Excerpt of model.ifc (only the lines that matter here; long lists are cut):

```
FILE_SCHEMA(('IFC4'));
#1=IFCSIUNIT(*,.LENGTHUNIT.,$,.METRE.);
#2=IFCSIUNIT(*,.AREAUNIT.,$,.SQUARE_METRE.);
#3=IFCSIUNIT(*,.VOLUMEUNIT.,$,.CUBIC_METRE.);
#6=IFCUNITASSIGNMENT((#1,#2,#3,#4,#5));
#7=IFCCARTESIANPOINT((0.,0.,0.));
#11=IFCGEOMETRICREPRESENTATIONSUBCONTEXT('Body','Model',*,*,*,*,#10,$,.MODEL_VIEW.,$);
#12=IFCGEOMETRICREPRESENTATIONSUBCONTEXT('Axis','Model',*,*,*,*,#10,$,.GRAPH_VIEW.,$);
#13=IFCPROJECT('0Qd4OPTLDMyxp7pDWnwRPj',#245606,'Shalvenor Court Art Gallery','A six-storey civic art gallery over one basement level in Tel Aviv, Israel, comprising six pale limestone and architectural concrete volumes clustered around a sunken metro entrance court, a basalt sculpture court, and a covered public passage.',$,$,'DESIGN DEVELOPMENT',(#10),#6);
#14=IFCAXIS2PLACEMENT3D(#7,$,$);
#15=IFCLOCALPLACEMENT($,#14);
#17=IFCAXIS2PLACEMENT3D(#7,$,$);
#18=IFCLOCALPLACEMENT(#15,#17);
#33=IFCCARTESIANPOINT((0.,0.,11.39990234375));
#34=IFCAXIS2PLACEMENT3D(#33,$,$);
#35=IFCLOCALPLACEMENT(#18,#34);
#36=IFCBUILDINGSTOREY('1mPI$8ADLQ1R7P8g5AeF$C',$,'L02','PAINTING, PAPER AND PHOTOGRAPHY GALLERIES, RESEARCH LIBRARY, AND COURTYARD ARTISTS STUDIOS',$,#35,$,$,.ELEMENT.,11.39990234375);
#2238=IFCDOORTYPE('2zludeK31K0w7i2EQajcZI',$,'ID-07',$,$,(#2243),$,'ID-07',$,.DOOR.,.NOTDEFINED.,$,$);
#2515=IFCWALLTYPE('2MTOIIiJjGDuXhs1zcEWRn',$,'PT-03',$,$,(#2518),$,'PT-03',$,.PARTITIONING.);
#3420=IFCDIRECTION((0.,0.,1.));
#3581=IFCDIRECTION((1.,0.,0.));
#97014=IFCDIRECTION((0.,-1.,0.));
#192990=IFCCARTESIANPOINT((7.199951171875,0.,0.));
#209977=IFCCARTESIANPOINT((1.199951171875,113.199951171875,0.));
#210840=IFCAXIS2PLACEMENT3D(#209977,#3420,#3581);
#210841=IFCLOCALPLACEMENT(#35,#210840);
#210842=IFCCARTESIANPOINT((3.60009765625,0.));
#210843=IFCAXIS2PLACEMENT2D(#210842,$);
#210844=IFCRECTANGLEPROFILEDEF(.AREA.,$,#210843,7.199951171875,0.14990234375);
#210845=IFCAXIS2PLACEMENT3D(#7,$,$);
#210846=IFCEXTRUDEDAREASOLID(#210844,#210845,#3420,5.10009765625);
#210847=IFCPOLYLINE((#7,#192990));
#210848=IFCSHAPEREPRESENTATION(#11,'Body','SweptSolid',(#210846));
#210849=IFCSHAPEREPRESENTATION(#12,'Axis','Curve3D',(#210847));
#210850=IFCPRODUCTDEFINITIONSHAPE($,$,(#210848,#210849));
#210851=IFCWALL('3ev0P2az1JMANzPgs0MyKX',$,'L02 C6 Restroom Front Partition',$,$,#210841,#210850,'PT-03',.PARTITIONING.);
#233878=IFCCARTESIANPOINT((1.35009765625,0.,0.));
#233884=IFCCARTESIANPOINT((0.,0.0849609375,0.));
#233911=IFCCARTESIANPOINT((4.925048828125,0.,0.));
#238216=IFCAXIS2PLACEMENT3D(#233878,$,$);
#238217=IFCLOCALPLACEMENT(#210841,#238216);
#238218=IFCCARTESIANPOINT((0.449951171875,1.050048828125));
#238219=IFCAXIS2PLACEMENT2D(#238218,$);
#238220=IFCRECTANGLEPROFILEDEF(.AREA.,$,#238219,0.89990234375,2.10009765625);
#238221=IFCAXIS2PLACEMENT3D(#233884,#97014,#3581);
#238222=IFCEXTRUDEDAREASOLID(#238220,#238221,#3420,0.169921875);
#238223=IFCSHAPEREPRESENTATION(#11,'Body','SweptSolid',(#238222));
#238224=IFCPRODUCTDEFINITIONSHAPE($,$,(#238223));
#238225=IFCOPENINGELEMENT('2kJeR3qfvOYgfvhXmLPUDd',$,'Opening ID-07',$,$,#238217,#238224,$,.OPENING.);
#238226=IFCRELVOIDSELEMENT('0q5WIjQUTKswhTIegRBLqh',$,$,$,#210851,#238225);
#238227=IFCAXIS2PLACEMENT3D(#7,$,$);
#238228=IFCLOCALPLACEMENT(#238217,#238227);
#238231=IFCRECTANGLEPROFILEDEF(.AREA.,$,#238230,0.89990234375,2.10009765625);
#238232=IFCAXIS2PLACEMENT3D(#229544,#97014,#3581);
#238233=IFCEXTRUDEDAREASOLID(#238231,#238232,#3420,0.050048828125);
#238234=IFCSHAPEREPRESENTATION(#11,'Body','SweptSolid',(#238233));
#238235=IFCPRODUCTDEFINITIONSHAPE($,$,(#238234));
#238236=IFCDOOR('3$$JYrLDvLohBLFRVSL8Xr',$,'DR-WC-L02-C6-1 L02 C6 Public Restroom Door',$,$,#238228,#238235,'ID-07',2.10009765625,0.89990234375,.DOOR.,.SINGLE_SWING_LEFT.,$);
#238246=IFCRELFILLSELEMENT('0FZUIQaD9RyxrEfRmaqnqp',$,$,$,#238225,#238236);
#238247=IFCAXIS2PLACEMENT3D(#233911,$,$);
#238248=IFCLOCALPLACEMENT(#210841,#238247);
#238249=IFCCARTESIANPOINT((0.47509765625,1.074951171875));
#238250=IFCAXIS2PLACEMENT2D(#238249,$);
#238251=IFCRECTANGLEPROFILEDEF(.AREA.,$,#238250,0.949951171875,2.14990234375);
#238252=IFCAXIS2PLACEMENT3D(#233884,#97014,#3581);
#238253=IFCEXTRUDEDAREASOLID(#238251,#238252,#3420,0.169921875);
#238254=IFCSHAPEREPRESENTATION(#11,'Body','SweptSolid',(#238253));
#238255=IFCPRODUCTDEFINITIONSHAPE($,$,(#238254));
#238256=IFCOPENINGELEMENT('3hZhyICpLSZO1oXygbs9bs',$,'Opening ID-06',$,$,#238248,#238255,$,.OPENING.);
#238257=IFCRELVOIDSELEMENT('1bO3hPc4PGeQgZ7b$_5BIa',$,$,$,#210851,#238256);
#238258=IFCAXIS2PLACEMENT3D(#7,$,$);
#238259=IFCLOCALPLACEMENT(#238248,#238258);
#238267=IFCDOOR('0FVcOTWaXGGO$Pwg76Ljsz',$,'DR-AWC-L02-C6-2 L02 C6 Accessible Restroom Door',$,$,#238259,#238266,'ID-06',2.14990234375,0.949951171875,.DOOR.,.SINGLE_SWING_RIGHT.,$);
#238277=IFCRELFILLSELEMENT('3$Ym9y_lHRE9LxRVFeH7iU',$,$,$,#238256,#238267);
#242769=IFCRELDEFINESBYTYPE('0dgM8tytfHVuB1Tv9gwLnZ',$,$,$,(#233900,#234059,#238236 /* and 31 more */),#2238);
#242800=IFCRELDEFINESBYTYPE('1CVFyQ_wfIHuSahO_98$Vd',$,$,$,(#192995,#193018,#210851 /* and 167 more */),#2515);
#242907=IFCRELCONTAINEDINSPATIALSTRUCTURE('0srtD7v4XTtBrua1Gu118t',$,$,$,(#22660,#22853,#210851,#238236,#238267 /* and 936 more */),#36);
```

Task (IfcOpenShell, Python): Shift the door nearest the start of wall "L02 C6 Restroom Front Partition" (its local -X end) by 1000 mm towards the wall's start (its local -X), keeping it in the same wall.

```python
import ifcopenshell
import ifcopenshell.api.geometry
import ifcopenshell.util.placement

model = ifcopenshell.open("model.ifc")

door = model.by_id(238236)
opening = door.FillsVoids[0].RelatingOpeningElement
wall = opening.VoidsElements[0].RelatingBuildingElement

wall_matrix = ifcopenshell.util.placement.get_local_placement(wall.ObjectPlacement)
shift = wall_matrix[:3, 0] * -1.0
before = ifcopenshell.util.placement.get_local_placement(door.ObjectPlacement)[:3, 3].copy()

# The door is placed relative to its opening, so it follows when the opening moves.
matrix = ifcopenshell.util.placement.get_local_placement(opening.ObjectPlacement)
matrix[:3, 3] += shift
ifcopenshell.api.geometry.edit_object_placement(
    model, product=opening, matrix=matrix, is_si=False, should_transform_children=True
)

after = ifcopenshell.util.placement.get_local_placement(door.ObjectPlacement)[:3, 3]
print("door moved by", (after - before).round(3) + 0.0)

model.write("model-out.ifc")
```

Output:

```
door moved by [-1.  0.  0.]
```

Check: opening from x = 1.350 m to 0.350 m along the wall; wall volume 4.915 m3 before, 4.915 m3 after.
